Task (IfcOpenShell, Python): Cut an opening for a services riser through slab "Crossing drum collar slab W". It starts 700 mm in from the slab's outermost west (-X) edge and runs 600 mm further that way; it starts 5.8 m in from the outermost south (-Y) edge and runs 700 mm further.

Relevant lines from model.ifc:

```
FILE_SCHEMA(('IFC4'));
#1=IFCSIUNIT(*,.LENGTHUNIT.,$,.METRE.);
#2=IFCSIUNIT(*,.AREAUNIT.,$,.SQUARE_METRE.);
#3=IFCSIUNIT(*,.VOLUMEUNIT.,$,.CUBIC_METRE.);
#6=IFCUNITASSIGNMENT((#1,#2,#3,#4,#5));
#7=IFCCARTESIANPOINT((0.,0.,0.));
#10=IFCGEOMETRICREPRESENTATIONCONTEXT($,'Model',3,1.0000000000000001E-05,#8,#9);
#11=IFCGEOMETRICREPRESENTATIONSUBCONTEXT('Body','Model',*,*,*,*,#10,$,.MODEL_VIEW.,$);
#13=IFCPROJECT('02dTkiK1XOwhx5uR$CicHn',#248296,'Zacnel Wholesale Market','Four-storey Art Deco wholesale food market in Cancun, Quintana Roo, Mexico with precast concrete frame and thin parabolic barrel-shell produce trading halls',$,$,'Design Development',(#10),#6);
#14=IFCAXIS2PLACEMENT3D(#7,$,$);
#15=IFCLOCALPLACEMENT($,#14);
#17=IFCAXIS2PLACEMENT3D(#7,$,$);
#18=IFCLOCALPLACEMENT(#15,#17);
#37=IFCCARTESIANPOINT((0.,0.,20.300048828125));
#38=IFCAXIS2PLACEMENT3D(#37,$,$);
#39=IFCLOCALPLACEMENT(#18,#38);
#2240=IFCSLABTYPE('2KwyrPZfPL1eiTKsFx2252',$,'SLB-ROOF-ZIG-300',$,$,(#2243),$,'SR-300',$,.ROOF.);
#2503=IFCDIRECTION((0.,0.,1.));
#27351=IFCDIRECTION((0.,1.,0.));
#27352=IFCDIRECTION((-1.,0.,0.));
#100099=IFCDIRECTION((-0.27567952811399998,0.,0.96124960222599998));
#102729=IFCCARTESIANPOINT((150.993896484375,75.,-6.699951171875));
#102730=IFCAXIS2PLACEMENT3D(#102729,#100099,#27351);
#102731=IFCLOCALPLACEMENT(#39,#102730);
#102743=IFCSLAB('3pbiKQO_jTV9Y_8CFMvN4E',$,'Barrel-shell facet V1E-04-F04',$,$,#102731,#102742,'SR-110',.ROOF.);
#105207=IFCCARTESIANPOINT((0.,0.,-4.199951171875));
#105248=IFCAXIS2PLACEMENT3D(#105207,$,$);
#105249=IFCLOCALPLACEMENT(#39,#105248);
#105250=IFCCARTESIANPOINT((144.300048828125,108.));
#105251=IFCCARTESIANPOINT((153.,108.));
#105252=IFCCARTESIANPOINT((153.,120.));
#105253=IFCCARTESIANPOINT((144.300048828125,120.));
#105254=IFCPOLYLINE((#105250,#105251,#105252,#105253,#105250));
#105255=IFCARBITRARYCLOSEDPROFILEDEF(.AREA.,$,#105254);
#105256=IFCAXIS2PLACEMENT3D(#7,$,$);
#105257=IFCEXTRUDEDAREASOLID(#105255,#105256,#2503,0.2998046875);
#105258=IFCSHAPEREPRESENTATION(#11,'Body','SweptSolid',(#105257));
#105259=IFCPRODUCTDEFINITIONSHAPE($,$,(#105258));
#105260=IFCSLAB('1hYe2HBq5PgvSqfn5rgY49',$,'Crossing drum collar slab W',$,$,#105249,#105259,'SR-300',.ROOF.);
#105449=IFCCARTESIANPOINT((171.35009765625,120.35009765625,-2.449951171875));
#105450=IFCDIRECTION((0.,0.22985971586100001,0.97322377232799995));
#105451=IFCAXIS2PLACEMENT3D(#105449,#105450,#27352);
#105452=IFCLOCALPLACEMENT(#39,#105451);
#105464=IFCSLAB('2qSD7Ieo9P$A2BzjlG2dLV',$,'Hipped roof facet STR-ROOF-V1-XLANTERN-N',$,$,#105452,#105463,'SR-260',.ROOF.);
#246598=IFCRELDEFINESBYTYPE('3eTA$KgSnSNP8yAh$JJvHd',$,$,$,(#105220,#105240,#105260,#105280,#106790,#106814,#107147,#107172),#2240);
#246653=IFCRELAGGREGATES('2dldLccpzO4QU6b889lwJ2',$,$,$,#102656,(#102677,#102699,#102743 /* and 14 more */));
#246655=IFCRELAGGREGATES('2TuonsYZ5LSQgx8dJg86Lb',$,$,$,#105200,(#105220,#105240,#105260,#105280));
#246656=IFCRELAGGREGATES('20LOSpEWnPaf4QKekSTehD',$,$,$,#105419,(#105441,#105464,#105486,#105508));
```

```python
import numpy as np
import ifcopenshell
import ifcopenshell.api.feature
import ifcopenshell.api.geometry
import ifcopenshell.api.root
import ifcopenshell.geom
import ifcopenshell.util.placement
import ifcopenshell.util.representation
import ifcopenshell.util.shape
import ifcopenshell.util.unit

model = ifcopenshell.open("model.ifc")
unit_scale = ifcopenshell.util.unit.calculate_unit_scale(model)
settings = ifcopenshell.geom.settings()


def volume(element):
    """Net volume in cubic metres, openings subtracted."""
    shape = ifcopenshell.geom.create_shape(settings, element)
    return ifcopenshell.util.shape.get_volume(shape.geometry)


slab = model.by_guid("1hYe2HBq5PgvSqfn5rgY49")
before = volume(slab)

# Extent in the slab's own axes, in metres. The edges named are its -X and -Y sides.
slab_shape = ifcopenshell.geom.create_shape(settings, slab)
vertices = ifcopenshell.util.shape.get_vertices(slab_shape.geometry)
x_min, y_min, bottom = vertices.min(axis=0)
top = vertices[:, 2].max()

opening = ifcopenshell.api.root.create_entity(model, ifc_class="IfcOpeningElement", name="Services riser opening", predefined_type="OPENING")
context = ifcopenshell.util.representation.get_context(model, "Model", "Body", "MODEL_VIEW")
width, depth = 0.6, 0.7
outline = [(0.0, 0.0), (width, 0.0), (width, depth), (0.0, depth), (0.0, 0.0)]
# Overshoot both faces by 50 mm so the cut is clean.
shape = ifcopenshell.api.geometry.add_slab_representation(
    model, context=context, depth=top - bottom + 0.1, polyline=outline
)
ifcopenshell.api.geometry.assign_representation(model, product=opening, representation=shape)

matrix = ifcopenshell.util.placement.get_local_placement(slab.ObjectPlacement)
matrix[:, 3] = matrix @ np.append(np.array([x_min + 0.7, y_min + 5.8, bottom - 0.05]) / unit_scale, 1.0)
ifcopenshell.api.geometry.edit_object_placement(model, product=opening, matrix=matrix, is_si=False)
ifcopenshell.api.feature.add_feature(model, feature=opening, element=slab)

after = volume(slab)

print(f"slab volume {before:.3f} -> {after:.3f} m3")

model.write("model_rev.ifc")
```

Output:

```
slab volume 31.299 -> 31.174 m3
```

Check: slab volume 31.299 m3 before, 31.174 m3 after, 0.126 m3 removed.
